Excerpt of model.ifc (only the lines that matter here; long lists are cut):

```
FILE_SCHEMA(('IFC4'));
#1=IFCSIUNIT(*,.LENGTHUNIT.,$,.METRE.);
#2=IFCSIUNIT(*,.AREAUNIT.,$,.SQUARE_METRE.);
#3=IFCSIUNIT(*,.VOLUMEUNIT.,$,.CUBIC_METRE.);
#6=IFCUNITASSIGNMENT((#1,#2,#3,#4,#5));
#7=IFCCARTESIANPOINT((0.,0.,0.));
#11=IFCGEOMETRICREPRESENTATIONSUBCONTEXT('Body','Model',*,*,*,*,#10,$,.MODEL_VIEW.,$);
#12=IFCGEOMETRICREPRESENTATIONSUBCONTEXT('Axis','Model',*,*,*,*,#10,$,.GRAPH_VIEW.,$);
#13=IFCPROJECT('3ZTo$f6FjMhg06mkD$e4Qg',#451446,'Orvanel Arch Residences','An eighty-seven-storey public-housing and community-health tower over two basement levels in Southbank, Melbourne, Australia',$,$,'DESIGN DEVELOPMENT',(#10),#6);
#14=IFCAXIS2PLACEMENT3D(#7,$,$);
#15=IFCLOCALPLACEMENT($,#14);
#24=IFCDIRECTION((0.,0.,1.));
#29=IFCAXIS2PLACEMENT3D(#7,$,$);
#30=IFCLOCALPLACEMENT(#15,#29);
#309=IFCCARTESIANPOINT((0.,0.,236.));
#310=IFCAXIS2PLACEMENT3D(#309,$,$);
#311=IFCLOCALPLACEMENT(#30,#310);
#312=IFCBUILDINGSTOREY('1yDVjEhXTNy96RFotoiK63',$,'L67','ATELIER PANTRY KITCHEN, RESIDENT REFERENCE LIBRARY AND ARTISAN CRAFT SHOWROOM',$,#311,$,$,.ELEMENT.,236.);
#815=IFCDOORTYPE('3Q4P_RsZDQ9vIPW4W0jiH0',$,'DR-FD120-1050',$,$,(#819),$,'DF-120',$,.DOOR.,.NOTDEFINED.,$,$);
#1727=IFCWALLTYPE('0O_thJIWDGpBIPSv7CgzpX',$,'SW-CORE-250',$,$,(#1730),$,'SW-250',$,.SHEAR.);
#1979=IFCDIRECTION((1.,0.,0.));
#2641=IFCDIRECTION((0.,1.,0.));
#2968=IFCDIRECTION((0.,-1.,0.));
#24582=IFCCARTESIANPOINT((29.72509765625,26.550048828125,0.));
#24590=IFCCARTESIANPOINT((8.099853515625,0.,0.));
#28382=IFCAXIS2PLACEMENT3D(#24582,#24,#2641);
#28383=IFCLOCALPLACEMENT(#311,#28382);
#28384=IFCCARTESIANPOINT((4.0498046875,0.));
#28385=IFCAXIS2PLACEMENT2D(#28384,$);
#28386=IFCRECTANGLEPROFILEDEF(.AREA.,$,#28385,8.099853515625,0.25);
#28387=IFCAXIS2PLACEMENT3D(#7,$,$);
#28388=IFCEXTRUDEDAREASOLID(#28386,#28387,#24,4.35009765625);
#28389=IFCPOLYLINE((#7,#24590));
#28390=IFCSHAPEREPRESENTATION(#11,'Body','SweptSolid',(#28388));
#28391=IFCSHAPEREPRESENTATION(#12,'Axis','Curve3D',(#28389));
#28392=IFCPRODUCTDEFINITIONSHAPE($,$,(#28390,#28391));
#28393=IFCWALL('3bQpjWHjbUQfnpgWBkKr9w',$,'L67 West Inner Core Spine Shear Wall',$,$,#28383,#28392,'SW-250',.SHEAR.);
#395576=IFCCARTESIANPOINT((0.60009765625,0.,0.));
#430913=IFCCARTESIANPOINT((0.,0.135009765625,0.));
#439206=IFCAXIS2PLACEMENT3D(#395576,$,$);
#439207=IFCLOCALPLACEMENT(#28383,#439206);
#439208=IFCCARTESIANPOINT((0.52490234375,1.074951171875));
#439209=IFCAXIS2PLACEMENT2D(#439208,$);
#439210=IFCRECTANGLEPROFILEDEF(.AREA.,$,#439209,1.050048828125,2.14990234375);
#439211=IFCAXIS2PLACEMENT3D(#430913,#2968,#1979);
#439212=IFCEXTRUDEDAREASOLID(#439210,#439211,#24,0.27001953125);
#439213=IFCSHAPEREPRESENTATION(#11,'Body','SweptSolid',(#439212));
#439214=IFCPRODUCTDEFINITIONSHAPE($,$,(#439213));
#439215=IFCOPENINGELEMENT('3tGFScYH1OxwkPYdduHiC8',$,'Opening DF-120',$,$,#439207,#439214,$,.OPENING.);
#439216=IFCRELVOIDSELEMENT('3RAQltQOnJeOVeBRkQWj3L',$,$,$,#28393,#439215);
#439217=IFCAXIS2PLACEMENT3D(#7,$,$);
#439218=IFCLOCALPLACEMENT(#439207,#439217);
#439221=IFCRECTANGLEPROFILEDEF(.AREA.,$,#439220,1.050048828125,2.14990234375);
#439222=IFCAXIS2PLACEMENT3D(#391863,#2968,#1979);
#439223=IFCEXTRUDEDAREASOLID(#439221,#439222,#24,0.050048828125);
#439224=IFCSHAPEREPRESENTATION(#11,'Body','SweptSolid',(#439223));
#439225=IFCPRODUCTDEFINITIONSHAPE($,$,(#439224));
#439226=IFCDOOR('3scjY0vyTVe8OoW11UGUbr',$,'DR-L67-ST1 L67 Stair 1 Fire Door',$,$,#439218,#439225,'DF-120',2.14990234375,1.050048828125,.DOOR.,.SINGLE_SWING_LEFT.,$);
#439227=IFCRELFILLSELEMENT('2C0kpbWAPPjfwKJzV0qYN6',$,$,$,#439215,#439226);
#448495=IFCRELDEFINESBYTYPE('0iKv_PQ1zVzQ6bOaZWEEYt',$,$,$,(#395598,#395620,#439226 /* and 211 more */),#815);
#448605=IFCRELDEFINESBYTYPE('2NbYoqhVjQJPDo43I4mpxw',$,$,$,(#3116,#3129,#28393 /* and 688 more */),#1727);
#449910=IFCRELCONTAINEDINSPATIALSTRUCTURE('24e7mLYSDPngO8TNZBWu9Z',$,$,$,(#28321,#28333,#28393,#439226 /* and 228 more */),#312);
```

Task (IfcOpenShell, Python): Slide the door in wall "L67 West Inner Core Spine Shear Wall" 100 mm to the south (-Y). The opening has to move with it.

```python
import ifcopenshell
import ifcopenshell.api.geometry
import ifcopenshell.util.placement

model = ifcopenshell.open("model.ifc")

door = model.by_id(439226)
opening = door.FillsVoids[0].RelatingOpeningElement
wall = opening.VoidsElements[0].RelatingBuildingElement

wall_matrix = ifcopenshell.util.placement.get_local_placement(wall.ObjectPlacement)
shift = wall_matrix[:3, 0] * -0.1
before = ifcopenshell.util.placement.get_local_placement(door.ObjectPlacement)[:3, 3].copy()

# The door is placed relative to its opening, so it follows when the opening moves.
matrix = ifcopenshell.util.placement.get_local_placement(opening.ObjectPlacement)
matrix[:3, 3] += shift
ifcopenshell.api.geometry.edit_object_placement(
    model, product=opening, matrix=matrix, is_si=False, should_transform_children=True
)

after = ifcopenshell.util.placement.get_local_placement(door.ObjectPlacement)[:3, 3]
print("door moved by", (after - before).round(3) + 0.0)

model.write("model_v2.ifc")
```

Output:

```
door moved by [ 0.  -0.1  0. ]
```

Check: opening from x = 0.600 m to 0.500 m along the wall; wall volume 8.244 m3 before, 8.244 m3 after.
